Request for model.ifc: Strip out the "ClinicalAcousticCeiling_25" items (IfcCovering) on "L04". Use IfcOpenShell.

First a look at what the model holds.

```python
import ifcopenshell
import ifcopenshell.util.element

model = ifcopenshell.open("model.ifc")
print(model.schema)
storey = next(s for s in model.by_type("IfcBuildingStorey") if s.Name == "L04")
coverings = [e for e in ifcopenshell.util.element.get_decomposition(storey) if e.is_a("IfcCovering")]
seen = {}
for e in coverings:
    element_type = ifcopenshell.util.element.get_type(e)
    name = element_type.Name if element_type not in (None, e) else None
    seen[name] = seen.get(name, 0) + 1
for name, count in sorted(seen.items(), key=str):
    print(count, "x", name)
```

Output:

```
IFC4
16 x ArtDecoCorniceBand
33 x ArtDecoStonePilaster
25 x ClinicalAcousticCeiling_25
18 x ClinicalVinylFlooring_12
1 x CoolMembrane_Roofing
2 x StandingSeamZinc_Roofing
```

```python
import ifcopenshell
import ifcopenshell.api.root
import ifcopenshell.util.element

model = ifcopenshell.open("model.ifc")

storey = next(s for s in model.by_type("IfcBuildingStorey") if s.Name == "L04")
coverings = [e for e in ifcopenshell.util.element.get_decomposition(storey) if e.is_a("IfcCovering")]
targets = [e for e in coverings if (t := ifcopenshell.util.element.get_type(e)) not in (None, e) and t.Name == "ClinicalAcousticCeiling_25"]

for e in targets:
    ifcopenshell.api.root.remove_product(model, product=e)
print(len(targets), "removed")

model.write("model_v2.ifc")
```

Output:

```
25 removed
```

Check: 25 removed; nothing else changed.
